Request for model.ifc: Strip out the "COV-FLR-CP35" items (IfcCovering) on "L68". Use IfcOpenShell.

First a look at what the model holds.

```python
import ifcopenshell
import ifcopenshell.util.element

model = ifcopenshell.open("model.ifc")
print(model.schema)
storey = next(s for s in model.by_type("IfcBuildingStorey") if s.Name == "L68")
coverings = [e for e in ifcopenshell.util.element.get_decomposition(storey) if e.is_a("IfcCovering")]
seen = {}
for e in coverings:
    element_type = ifcopenshell.util.element.get_type(e)
    name = element_type.Name if element_type not in (None, e) else None
    seen[name] = seen.get(name, 0) + 1
for name, count in sorted(seen.items(), key=str):
    print(count, "x", name)
```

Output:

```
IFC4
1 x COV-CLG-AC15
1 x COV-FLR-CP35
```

```python
import ifcopenshell
import ifcopenshell.api.root
import ifcopenshell.util.element

model = ifcopenshell.open("model.ifc")

storey = next(s for s in model.by_type("IfcBuildingStorey") if s.Name == "L68")
coverings = [e for e in ifcopenshell.util.element.get_decomposition(storey) if e.is_a("IfcCovering")]
targets = [e for e in coverings if (t := ifcopenshell.util.element.get_type(e)) not in (None, e) and t.Name == "COV-FLR-CP35"]

for e in targets:
    ifcopenshell.api.root.remove_product(model, product=e)
print(len(targets), "removed")

model.write("model_updated.ifc")
```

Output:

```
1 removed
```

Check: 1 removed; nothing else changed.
